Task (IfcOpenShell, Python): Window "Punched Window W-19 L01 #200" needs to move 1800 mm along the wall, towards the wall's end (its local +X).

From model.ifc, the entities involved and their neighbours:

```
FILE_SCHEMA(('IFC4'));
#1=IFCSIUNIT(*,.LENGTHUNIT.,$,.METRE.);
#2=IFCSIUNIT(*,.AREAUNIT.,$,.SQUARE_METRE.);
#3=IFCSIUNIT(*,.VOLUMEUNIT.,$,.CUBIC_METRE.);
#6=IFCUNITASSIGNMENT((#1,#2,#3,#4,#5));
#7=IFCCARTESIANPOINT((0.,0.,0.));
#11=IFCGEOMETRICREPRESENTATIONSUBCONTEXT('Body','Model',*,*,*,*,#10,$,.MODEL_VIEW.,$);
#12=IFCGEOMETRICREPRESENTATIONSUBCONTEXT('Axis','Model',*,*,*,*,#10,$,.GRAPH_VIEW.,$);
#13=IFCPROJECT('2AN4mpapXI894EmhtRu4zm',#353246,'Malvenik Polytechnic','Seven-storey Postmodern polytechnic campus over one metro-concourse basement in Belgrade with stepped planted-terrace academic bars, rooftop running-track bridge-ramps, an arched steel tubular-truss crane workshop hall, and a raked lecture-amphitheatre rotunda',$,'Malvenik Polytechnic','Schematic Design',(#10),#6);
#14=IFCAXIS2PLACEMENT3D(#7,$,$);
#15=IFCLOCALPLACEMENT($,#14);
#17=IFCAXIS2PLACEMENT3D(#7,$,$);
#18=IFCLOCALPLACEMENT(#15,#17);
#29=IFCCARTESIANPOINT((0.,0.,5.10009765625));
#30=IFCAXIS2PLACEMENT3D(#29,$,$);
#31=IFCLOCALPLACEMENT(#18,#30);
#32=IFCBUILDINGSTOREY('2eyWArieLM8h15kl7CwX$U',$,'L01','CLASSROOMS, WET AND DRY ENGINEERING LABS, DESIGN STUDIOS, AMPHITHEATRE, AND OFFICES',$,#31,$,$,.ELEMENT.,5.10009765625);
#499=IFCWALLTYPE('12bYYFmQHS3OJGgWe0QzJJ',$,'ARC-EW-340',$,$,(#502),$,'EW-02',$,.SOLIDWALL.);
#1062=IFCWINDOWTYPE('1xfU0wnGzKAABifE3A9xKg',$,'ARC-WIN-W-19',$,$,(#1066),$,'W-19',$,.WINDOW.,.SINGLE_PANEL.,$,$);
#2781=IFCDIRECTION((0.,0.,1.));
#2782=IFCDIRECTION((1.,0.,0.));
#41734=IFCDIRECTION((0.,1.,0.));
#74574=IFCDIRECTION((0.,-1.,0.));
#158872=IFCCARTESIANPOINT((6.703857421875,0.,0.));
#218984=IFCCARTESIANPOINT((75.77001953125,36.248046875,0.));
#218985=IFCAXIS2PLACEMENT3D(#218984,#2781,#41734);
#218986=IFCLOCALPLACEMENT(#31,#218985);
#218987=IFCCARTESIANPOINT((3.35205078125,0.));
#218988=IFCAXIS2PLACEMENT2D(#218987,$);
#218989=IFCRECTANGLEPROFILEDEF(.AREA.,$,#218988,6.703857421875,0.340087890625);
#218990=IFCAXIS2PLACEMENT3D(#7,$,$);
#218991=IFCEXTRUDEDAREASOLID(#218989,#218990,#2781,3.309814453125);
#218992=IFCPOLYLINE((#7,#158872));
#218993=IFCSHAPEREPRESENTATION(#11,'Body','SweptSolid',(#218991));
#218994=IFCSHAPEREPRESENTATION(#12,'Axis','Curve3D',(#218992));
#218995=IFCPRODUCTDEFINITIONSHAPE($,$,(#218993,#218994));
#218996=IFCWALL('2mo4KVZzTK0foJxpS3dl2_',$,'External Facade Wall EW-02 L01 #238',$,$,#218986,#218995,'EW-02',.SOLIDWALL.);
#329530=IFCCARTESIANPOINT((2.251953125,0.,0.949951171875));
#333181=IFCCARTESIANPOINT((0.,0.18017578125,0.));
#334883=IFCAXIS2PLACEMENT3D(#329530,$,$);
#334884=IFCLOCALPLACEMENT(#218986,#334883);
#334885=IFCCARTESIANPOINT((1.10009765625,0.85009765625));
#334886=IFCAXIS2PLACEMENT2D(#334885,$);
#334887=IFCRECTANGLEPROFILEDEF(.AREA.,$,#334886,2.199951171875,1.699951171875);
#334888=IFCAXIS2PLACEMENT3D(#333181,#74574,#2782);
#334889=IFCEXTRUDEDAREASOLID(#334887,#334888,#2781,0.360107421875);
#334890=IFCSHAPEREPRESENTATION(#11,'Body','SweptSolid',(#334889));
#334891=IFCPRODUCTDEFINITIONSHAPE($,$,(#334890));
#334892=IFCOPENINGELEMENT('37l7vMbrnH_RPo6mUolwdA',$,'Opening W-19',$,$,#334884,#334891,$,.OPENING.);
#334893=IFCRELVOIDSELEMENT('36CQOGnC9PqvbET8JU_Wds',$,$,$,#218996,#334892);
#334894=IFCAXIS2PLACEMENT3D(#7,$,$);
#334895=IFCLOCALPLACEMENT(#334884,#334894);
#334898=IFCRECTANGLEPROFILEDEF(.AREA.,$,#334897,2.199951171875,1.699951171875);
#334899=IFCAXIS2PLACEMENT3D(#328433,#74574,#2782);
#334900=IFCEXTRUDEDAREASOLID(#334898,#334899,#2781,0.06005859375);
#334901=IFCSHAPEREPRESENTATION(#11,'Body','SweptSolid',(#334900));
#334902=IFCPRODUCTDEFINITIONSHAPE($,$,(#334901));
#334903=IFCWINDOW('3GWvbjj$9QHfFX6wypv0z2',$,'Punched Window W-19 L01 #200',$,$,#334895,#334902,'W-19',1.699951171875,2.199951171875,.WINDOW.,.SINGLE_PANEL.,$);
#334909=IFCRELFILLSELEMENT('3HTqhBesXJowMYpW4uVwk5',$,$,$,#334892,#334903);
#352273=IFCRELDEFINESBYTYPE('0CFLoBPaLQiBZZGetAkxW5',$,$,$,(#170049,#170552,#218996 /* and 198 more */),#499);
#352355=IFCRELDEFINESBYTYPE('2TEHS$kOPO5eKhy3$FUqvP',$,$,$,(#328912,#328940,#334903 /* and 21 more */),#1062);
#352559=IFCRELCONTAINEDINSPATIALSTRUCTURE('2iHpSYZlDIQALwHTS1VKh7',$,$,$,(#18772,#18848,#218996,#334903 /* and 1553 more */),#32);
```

```python
import ifcopenshell
import ifcopenshell.api.geometry
import ifcopenshell.util.placement
import ifcopenshell.util.unit

model = ifcopenshell.open("model.ifc")
unit_scale = ifcopenshell.util.unit.calculate_unit_scale(model)

window = model.by_id(334903)
opening = window.FillsVoids[0].RelatingOpeningElement
wall = opening.VoidsElements[0].RelatingBuildingElement

wall_matrix = ifcopenshell.util.placement.get_local_placement(wall.ObjectPlacement)
shift = wall_matrix[:3, 0] * 1.8 / unit_scale
before = ifcopenshell.util.placement.get_local_placement(window.ObjectPlacement)[:3, 3].copy()

# The window is placed relative to its opening, so it follows when the opening moves.
matrix = ifcopenshell.util.placement.get_local_placement(opening.ObjectPlacement)
matrix[:3, 3] += shift
ifcopenshell.api.geometry.edit_object_placement(
    model, product=opening, matrix=matrix, is_si=False, should_transform_children=True
)

after = ifcopenshell.util.placement.get_local_placement(window.ObjectPlacement)[:3, 3]
print("window moved by", (after - before).round(3) + 0.0)

model.write("model_rev.ifc")
```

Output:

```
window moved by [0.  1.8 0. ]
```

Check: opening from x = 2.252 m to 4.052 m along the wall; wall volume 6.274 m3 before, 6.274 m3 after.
